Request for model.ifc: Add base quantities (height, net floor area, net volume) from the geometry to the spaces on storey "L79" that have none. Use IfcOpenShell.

First a look at what the model holds.

```python
import ifcopenshell
import ifcopenshell.util.element
import ifcopenshell.util.unit

model = ifcopenshell.open("model.ifc")
print(model.schema)
for unit_type in ("LENGTHUNIT", "AREAUNIT", "VOLUMEUNIT"):
    print(unit_type, ifcopenshell.util.unit.calculate_unit_scale(model, unit_type))
storey = next(s for s in model.by_type("IfcBuildingStorey") if s.Name == "L79")
spaces = [e for e in ifcopenshell.util.element.get_decomposition(storey) if e.is_a("IfcSpace")]
for e in sorted(spaces, key=lambda e: e.id()):
    print(e.id(), e.is_a(), e.Name, list(ifcopenshell.util.element.get_psets(e, qtos_only=True)), sep=" | ")
```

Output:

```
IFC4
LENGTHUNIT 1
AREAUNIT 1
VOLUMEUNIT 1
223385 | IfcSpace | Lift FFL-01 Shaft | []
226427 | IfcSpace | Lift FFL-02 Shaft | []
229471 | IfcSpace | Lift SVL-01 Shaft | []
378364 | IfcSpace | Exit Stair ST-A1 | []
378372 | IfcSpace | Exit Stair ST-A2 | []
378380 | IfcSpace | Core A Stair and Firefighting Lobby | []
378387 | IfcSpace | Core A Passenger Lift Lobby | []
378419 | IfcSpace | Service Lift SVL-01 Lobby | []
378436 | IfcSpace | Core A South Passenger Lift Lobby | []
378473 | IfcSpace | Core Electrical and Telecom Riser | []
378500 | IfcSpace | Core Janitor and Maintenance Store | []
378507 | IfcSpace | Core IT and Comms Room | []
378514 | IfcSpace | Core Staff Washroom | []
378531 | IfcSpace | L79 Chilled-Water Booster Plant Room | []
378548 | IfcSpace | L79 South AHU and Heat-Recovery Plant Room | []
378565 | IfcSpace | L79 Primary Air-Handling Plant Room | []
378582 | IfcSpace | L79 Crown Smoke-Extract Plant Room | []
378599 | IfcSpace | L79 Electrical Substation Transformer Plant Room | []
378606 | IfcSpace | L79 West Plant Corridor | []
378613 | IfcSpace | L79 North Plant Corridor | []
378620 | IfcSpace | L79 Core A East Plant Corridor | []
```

```python
import ifcopenshell
import ifcopenshell.api.pset
import ifcopenshell.geom
import ifcopenshell.util.element
import ifcopenshell.util.shape
import ifcopenshell.util.unit

model = ifcopenshell.open("model.ifc")
unit_scale = ifcopenshell.util.unit.calculate_unit_scale(model)
area_scale = ifcopenshell.util.unit.calculate_unit_scale(model, "AREAUNIT")
volume_scale = ifcopenshell.util.unit.calculate_unit_scale(model, "VOLUMEUNIT")
settings = ifcopenshell.geom.settings()

storey = next(s for s in model.by_type("IfcBuildingStorey") if s.Name == "L79")
spaces = [e for e in ifcopenshell.util.element.get_decomposition(storey) if e.is_a("IfcSpace")]

for e in sorted(spaces, key=lambda e: e.id()):
    if ifcopenshell.util.element.get_psets(e, qtos_only=True, should_inherit=False):
        continue
    # Geometry comes back in metres, in the element's own axes.
    shape = ifcopenshell.geom.create_shape(settings, e)
    values = {
        "Height": ifcopenshell.util.shape.get_z(shape.geometry) / unit_scale,
        "NetFloorArea": ifcopenshell.util.shape.get_footprint_area(shape.geometry) / area_scale,
        "NetVolume": ifcopenshell.util.shape.get_volume(shape.geometry) / volume_scale,
    }
    qto = ifcopenshell.api.pset.add_qto(model, product=e, name="Qto_SpaceBaseQuantities")
    ifcopenshell.api.pset.edit_qto(model, qto=qto, properties=values)
    print(e.id(), {k: round(v, 3) for k, v in values.items()})

model.write("model_v2.ifc")
```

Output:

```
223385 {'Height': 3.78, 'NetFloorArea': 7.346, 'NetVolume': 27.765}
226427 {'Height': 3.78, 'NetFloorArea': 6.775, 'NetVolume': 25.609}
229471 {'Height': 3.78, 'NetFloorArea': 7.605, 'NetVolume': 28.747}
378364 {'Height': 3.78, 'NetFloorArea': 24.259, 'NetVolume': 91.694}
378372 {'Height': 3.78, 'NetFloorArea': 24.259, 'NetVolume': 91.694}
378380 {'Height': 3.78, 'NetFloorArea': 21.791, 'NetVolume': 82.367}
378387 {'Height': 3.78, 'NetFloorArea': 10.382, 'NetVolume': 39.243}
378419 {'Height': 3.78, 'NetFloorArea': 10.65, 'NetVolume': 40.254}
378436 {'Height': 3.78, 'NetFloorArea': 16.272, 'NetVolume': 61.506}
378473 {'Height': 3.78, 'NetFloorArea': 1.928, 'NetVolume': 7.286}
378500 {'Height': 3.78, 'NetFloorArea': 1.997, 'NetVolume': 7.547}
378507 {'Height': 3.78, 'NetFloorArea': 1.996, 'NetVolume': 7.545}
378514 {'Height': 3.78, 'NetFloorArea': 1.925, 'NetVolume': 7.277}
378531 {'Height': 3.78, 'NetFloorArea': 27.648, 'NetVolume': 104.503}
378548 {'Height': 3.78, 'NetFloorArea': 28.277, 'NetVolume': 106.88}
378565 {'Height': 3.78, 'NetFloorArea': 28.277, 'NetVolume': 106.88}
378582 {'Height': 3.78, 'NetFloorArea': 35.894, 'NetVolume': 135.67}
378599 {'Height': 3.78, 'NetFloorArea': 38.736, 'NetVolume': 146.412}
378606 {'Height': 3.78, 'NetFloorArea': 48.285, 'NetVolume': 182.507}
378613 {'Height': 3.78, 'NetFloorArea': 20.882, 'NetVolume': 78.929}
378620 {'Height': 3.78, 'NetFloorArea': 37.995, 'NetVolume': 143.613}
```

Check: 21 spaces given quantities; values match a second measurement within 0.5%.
